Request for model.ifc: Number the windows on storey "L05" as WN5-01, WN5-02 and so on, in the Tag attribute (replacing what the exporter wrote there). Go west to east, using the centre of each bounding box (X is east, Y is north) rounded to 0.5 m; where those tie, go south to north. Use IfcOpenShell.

First a look at what the model holds.

```python
import ifcopenshell
import ifcopenshell.util.element
import ifcopenshell.util.placement

model = ifcopenshell.open("model.ifc")
print(model.schema)
storey = next(s for s in model.by_type("IfcBuildingStorey") if s.Name == "L05")
windows = [e for e in ifcopenshell.util.element.get_decomposition(storey) if e.is_a("IfcWindow")]
for e in sorted(windows, key=lambda e: e.id()):
    origin = ifcopenshell.util.placement.get_local_placement(e.ObjectPlacement)[:3, 3]
    print(e.id(), e.Tag, e.Name, origin.round(2) + 0.0, sep=" | ")
```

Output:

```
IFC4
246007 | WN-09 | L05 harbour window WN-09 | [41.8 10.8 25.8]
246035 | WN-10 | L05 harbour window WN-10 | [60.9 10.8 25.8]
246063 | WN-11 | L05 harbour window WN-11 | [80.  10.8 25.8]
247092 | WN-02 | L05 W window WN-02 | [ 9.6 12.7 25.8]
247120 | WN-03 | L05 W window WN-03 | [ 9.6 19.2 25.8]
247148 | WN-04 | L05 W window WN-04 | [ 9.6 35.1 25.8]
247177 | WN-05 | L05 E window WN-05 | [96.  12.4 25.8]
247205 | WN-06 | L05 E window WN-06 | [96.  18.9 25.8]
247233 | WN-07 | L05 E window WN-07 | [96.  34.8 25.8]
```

```python
import ifcopenshell
import ifcopenshell.geom
import ifcopenshell.util.element
import ifcopenshell.util.shape

model = ifcopenshell.open("model.ifc")
settings = ifcopenshell.geom.settings()
settings.set("use-world-coords", True)


def centre(element):
    shape = ifcopenshell.geom.create_shape(settings, element)
    return ifcopenshell.util.shape.get_bbox_centroid(shape.geometry)


storey = next(s for s in model.by_type("IfcBuildingStorey") if s.Name == "L05")
windows = [e for e in ifcopenshell.util.element.get_decomposition(storey) if e.is_a("IfcWindow")]

# Insertion points can sit at a corner or the storey origin, so sort by the geometry (in metres).
centres = {e: centre(e) for e in windows}
windows.sort(key=lambda e: (round(centres[e][0] / 0.5), centres[e][1]))

for i, e in enumerate(windows, start=1):
    number = f"WN5-{i:02d}"
    e.Tag = number
    print(e.id(), number)

model.write("model-out.ifc")
```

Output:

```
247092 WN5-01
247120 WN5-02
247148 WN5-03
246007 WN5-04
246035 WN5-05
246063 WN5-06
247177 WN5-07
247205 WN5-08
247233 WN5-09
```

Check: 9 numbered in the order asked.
